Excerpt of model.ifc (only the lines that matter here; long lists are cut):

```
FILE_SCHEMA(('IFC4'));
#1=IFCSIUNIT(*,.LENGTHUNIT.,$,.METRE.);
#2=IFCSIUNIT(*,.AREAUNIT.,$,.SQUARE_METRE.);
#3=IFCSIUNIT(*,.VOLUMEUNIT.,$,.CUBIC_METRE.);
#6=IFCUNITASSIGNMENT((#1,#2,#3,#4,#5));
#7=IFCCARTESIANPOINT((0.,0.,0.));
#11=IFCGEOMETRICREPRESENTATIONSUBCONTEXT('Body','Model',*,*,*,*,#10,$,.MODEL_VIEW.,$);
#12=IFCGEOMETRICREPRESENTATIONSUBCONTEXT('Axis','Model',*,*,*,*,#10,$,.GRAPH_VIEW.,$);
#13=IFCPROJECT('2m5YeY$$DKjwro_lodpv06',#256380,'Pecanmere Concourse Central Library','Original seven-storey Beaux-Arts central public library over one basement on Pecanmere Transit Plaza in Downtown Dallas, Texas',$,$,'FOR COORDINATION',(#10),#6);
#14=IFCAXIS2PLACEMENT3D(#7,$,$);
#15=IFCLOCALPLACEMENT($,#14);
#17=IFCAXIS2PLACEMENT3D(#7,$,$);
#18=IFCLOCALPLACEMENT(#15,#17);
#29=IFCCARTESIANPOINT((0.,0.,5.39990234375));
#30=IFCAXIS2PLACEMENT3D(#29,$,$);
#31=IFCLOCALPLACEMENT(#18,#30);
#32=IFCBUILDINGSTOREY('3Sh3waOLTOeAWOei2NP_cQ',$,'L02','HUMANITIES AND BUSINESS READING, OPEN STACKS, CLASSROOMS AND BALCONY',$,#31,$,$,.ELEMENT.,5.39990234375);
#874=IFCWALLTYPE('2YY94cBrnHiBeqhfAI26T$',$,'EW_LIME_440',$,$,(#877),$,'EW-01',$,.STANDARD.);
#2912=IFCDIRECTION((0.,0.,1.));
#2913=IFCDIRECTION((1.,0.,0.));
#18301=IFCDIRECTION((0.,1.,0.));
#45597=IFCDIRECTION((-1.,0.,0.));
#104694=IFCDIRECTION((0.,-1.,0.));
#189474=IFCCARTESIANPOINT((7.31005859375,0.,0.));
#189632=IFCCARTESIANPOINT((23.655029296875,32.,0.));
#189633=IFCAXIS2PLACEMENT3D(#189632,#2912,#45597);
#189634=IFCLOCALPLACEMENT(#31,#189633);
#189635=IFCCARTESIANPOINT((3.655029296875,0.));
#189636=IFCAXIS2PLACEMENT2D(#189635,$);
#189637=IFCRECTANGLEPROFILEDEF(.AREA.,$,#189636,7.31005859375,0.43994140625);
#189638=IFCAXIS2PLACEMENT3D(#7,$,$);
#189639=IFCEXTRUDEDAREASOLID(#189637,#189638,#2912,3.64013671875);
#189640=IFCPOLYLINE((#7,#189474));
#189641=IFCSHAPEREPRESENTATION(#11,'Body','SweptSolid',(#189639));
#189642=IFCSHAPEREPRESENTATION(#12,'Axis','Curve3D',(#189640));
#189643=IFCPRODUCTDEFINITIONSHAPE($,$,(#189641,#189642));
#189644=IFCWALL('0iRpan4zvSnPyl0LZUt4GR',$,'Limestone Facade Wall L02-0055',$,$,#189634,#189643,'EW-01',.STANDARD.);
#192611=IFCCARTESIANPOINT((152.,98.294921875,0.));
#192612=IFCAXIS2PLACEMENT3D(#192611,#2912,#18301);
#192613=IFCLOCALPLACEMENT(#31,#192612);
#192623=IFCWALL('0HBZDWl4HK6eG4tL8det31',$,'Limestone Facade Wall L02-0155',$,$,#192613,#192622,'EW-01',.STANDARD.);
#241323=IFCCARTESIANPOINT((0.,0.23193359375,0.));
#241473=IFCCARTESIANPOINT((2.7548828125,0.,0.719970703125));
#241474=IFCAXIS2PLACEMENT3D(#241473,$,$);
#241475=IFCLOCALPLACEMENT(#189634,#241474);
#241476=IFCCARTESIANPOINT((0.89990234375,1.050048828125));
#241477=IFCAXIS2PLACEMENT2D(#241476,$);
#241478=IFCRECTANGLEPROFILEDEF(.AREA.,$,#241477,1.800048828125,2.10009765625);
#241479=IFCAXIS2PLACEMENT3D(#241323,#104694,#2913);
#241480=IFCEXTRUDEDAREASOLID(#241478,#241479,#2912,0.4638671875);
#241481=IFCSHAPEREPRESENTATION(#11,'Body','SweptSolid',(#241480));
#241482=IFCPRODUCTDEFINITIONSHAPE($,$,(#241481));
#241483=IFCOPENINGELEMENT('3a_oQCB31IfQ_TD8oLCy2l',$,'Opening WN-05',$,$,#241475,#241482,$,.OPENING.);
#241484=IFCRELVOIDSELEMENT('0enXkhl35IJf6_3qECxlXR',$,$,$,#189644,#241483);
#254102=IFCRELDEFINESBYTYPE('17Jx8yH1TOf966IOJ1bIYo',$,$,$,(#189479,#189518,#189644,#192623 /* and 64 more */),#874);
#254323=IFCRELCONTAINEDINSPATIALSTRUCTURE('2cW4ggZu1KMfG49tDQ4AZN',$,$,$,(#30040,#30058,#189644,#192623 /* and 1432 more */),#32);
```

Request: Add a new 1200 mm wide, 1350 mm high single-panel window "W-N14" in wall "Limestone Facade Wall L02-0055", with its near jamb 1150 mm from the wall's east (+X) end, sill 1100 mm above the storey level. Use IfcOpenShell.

```python
import numpy as np
import ifcopenshell
import ifcopenshell.api.feature
import ifcopenshell.api.geometry
import ifcopenshell.api.root
import ifcopenshell.api.spatial
import ifcopenshell.geom
import ifcopenshell.util.element
import ifcopenshell.util.placement
import ifcopenshell.util.representation
import ifcopenshell.util.shape
import ifcopenshell.util.unit

model = ifcopenshell.open("model.ifc")
unit_scale = ifcopenshell.util.unit.calculate_unit_scale(model)
settings = ifcopenshell.geom.settings()


def volume(element):
    """Net volume in cubic metres, openings subtracted."""
    shape = ifcopenshell.geom.create_shape(settings, element)
    return ifcopenshell.util.shape.get_volume(shape.geometry)


wall = model.by_id(189644)
storey = ifcopenshell.util.element.get_container(wall, ifc_class="IfcBuildingStorey")
context = ifcopenshell.util.representation.get_context(model, "Model", "Body", "MODEL_VIEW")
before = volume(wall)

width, height, from_end, sill = 1.2, 1.35, 1.15, 1.1  # metres

# The wall runs along its own X axis, and the end named is its -X end.
wall_shape = ifcopenshell.geom.create_shape(settings, wall)
x, y, z = ifcopenshell.util.shape.get_vertices(wall_shape.geometry).T
start = x.min() + from_end
face, thickness = float(y.min()), float(y.max() - y.min())
wall_matrix = ifcopenshell.util.placement.get_local_placement(wall.ObjectPlacement)
level = ifcopenshell.util.placement.get_local_placement(storey.ObjectPlacement)[2, 3]


def in_wall(x, y):
    """Placement at x, y metres in the wall's axes, at sill height."""
    matrix = wall_matrix.copy()
    matrix[:, 3] = wall_matrix @ np.array([x / unit_scale, y / unit_scale, 0.0, 1.0])
    matrix[2, 3] = level + sill / unit_scale
    return matrix


# Opening: a box that overshoots both wall faces by 50 mm.
opening = ifcopenshell.api.root.create_entity(model, ifc_class="IfcOpeningElement", predefined_type="OPENING")
box = ifcopenshell.api.geometry.add_wall_representation(
    model, context=context, length=width, height=height, thickness=thickness + 0.1
)
ifcopenshell.api.geometry.assign_representation(model, product=opening, representation=box)
ifcopenshell.api.geometry.edit_object_placement(model, product=opening, matrix=in_wall(start, face - 0.05), is_si=False)
ifcopenshell.api.feature.add_feature(model, feature=opening, element=wall)

window = ifcopenshell.api.root.create_entity(model, ifc_class="IfcWindow", name="W-N14", predefined_type="WINDOW")
window.OverallWidth, window.OverallHeight = width / unit_scale, height / unit_scale
window.PartitioningType = "SINGLE_PANEL"
body = ifcopenshell.api.geometry.add_window_representation(
    model,
    context=context,
    overall_width=window.OverallWidth,
    overall_height=window.OverallHeight,
    partition_type="SINGLE_PANEL",
)
ifcopenshell.api.geometry.assign_representation(model, product=window, representation=body)
ifcopenshell.api.spatial.assign_container(model, products=[window], relating_structure=storey)
ifcopenshell.api.feature.add_filling(model, opening=opening, element=window)

# Centre the window in the wall's thickness.
ifcopenshell.api.geometry.edit_object_placement(model, product=window, matrix=in_wall(start, face), is_si=False)
window_shape = ifcopenshell.geom.create_shape(settings, window)
depth = ifcopenshell.util.shape.get_vertices(window_shape.geometry)[:, 1]
offset = face + thickness / 2 - (depth.min() + depth.max()) / 2
ifcopenshell.api.geometry.edit_object_placement(model, product=window, matrix=in_wall(start, offset), is_si=False)

after = volume(wall)

print(f"wall volume {before:.3f} -> {after:.3f} m3")

model.write("model_updated.ifc")
```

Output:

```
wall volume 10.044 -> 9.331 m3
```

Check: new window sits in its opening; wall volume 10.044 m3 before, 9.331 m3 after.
